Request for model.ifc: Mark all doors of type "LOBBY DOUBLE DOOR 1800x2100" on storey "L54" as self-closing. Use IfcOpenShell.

First a look at what the model holds.

```python
import ifcopenshell
import ifcopenshell.util.element

model = ifcopenshell.open("model.ifc")
print(model.schema)
storey = next(s for s in model.by_type("IfcBuildingStorey") if s.Name == "L54")
doors = [e for e in ifcopenshell.util.element.get_decomposition(storey) if e.is_a("IfcDoor")]
seen = {}
for e in doors:
    element_type = ifcopenshell.util.element.get_type(e)
    key = (element_type.Name if element_type != e and element_type else None, ifcopenshell.util.element.get_pset(e, "Pset_DoorCommon", "SelfClosing"))
    seen[key] = seen.get(key, 0) + 1
for (name, value), count in sorted(seen.items(), key=str):
    print(count, "x", name, "|", value)
```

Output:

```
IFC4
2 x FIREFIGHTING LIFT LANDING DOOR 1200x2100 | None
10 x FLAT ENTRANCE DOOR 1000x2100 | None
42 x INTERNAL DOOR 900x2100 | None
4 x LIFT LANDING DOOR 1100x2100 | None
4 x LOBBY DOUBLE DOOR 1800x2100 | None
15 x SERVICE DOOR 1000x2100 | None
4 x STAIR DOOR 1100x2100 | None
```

```python
import ifcopenshell
import ifcopenshell.api.pset
import ifcopenshell.util.element

model = ifcopenshell.open("model.ifc")

storey = next(s for s in model.by_type("IfcBuildingStorey") if s.Name == "L54")
doors = [e for e in ifcopenshell.util.element.get_decomposition(storey) if e.is_a("IfcDoor")]

count = 0
for e in doors:
    element_type = ifcopenshell.util.element.get_type(e)
    if element_type in (None, e) or element_type.Name != "LOBBY DOUBLE DOOR 1800x2100":
        continue
    found = ifcopenshell.util.element.get_pset(e, "Pset_DoorCommon", should_inherit=False)
    if found:
        pset = model.by_id(found["id"])
        if len(ifcopenshell.util.element.get_elements_by_pset(pset)) > 1:
            pset = ifcopenshell.api.pset.unshare_pset(model, products=[e], pset=pset)[0]
    else:
        pset = ifcopenshell.api.pset.add_pset(model, product=e, name="Pset_DoorCommon")
    ifcopenshell.api.pset.edit_pset(model, pset=pset, properties={"SelfClosing": True})
    count += 1

print(count, "doors updated")

model.write("model_updated.ifc")
```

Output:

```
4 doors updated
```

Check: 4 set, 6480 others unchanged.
